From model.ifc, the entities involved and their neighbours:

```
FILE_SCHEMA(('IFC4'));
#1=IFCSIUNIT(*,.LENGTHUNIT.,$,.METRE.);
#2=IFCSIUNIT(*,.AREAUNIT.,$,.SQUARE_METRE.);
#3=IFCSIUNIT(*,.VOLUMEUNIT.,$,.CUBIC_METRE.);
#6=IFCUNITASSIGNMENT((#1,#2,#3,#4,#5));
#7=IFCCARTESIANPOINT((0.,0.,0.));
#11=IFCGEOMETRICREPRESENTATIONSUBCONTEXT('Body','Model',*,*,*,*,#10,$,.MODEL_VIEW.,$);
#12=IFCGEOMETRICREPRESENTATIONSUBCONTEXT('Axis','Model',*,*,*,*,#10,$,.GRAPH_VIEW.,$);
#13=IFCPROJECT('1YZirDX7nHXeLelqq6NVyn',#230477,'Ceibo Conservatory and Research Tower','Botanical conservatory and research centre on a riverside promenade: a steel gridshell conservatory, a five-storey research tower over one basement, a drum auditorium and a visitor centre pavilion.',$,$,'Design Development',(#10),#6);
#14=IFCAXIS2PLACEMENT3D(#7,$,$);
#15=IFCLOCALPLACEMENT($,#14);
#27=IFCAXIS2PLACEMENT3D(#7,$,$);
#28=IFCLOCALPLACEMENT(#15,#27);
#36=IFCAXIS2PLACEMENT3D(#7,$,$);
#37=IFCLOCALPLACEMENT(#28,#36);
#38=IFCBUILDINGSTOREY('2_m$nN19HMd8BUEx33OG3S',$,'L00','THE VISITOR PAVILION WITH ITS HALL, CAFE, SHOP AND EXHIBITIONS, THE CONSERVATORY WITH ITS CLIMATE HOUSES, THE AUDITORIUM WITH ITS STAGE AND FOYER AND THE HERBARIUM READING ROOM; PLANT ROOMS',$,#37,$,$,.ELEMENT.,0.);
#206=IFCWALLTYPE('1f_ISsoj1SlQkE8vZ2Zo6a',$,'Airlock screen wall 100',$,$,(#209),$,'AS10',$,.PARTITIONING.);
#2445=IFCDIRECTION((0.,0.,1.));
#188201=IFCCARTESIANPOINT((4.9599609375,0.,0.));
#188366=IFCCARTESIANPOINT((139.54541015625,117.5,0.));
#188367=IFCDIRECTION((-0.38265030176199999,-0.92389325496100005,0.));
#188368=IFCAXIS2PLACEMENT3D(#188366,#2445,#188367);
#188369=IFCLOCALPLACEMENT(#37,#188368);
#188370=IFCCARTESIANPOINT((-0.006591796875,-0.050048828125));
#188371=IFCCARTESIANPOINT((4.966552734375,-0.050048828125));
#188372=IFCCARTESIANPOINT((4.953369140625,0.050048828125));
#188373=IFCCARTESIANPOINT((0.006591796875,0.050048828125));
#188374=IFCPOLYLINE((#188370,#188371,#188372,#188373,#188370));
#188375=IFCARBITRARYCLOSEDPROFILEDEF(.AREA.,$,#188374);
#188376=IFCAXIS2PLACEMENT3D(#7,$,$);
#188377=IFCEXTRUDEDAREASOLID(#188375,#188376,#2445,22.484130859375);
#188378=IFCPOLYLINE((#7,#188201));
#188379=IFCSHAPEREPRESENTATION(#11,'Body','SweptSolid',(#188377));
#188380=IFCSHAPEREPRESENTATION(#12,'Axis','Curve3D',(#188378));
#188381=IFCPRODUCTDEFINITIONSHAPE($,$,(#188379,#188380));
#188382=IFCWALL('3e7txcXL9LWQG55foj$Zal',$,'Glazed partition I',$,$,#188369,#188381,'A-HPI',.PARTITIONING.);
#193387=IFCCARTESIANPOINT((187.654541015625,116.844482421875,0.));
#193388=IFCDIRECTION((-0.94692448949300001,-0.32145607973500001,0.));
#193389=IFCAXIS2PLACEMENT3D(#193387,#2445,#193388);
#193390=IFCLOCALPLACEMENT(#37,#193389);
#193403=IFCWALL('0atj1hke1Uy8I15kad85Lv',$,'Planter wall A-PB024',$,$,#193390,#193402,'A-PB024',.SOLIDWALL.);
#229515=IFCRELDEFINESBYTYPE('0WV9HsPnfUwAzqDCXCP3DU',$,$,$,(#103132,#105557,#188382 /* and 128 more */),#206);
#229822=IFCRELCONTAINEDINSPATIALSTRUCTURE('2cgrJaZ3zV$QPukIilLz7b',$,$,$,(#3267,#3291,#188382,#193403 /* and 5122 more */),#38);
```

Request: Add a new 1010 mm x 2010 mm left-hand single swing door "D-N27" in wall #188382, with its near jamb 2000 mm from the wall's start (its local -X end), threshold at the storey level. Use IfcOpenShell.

```python
import numpy as np
import ifcopenshell
import ifcopenshell.api.feature
import ifcopenshell.api.geometry
import ifcopenshell.api.root
import ifcopenshell.api.spatial
import ifcopenshell.geom
import ifcopenshell.util.element
import ifcopenshell.util.placement
import ifcopenshell.util.representation
import ifcopenshell.util.shape
import ifcopenshell.util.unit

model = ifcopenshell.open("model.ifc")
unit_scale = ifcopenshell.util.unit.calculate_unit_scale(model)
settings = ifcopenshell.geom.settings()


def volume(element):
    """Net volume in cubic metres, openings subtracted."""
    shape = ifcopenshell.geom.create_shape(settings, element)
    return ifcopenshell.util.shape.get_volume(shape.geometry)


wall = model.by_guid("3e7txcXL9LWQG55foj$Zal")
storey = ifcopenshell.util.element.get_container(wall, ifc_class="IfcBuildingStorey")
context = ifcopenshell.util.representation.get_context(model, "Model", "Body", "MODEL_VIEW")
before = volume(wall)

width, height, from_end, sill = 1.01, 2.01, 2, 0.0  # metres

# The wall runs along its own X axis, and the end named is its -X end.
wall_shape = ifcopenshell.geom.create_shape(settings, wall)
x, y, z = ifcopenshell.util.shape.get_vertices(wall_shape.geometry).T
start = x.min() + from_end
face, thickness = float(y.min()), float(y.max() - y.min())
wall_matrix = ifcopenshell.util.placement.get_local_placement(wall.ObjectPlacement)
level = ifcopenshell.util.placement.get_local_placement(storey.ObjectPlacement)[2, 3]


def in_wall(x, y):
    """Placement at x, y metres in the wall's axes, at sill height."""
    matrix = wall_matrix.copy()
    matrix[:, 3] = wall_matrix @ np.array([x / unit_scale, y / unit_scale, 0.0, 1.0])
    matrix[2, 3] = level + sill / unit_scale
    return matrix


# Opening: a box that overshoots both wall faces by 50 mm.
opening = ifcopenshell.api.root.create_entity(model, ifc_class="IfcOpeningElement", predefined_type="OPENING")
box = ifcopenshell.api.geometry.add_wall_representation(
    model, context=context, length=width, height=height, thickness=thickness + 0.1
)
ifcopenshell.api.geometry.assign_representation(model, product=opening, representation=box)
ifcopenshell.api.geometry.edit_object_placement(model, product=opening, matrix=in_wall(start, face - 0.05), is_si=False)
ifcopenshell.api.feature.add_feature(model, feature=opening, element=wall)

door = ifcopenshell.api.root.create_entity(model, ifc_class="IfcDoor", name="D-N27", predefined_type="DOOR")
door.OverallWidth, door.OverallHeight = width / unit_scale, height / unit_scale
door.OperationType = "SINGLE_SWING_LEFT"
body = ifcopenshell.api.geometry.add_door_representation(
    model,
    context=context,
    overall_width=door.OverallWidth,
    overall_height=door.OverallHeight,
    operation_type="SINGLE_SWING_LEFT",
    lining_properties={"LiningDepth": thickness / unit_scale, "ThresholdDepth": thickness / unit_scale},
)
ifcopenshell.api.geometry.assign_representation(model, product=door, representation=body)
ifcopenshell.api.spatial.assign_container(model, products=[door], relating_structure=storey)
ifcopenshell.api.feature.add_filling(model, opening=opening, element=door)

# The lining spans the wall, so the door starts at the wall face.
ifcopenshell.api.geometry.edit_object_placement(model, product=door, matrix=in_wall(start, face), is_si=False)

after = volume(wall)

print(f"wall volume {before:.3f} -> {after:.3f} m3")

model.write("model_edited.ifc")
```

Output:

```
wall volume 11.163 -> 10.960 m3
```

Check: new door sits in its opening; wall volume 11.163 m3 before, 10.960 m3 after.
